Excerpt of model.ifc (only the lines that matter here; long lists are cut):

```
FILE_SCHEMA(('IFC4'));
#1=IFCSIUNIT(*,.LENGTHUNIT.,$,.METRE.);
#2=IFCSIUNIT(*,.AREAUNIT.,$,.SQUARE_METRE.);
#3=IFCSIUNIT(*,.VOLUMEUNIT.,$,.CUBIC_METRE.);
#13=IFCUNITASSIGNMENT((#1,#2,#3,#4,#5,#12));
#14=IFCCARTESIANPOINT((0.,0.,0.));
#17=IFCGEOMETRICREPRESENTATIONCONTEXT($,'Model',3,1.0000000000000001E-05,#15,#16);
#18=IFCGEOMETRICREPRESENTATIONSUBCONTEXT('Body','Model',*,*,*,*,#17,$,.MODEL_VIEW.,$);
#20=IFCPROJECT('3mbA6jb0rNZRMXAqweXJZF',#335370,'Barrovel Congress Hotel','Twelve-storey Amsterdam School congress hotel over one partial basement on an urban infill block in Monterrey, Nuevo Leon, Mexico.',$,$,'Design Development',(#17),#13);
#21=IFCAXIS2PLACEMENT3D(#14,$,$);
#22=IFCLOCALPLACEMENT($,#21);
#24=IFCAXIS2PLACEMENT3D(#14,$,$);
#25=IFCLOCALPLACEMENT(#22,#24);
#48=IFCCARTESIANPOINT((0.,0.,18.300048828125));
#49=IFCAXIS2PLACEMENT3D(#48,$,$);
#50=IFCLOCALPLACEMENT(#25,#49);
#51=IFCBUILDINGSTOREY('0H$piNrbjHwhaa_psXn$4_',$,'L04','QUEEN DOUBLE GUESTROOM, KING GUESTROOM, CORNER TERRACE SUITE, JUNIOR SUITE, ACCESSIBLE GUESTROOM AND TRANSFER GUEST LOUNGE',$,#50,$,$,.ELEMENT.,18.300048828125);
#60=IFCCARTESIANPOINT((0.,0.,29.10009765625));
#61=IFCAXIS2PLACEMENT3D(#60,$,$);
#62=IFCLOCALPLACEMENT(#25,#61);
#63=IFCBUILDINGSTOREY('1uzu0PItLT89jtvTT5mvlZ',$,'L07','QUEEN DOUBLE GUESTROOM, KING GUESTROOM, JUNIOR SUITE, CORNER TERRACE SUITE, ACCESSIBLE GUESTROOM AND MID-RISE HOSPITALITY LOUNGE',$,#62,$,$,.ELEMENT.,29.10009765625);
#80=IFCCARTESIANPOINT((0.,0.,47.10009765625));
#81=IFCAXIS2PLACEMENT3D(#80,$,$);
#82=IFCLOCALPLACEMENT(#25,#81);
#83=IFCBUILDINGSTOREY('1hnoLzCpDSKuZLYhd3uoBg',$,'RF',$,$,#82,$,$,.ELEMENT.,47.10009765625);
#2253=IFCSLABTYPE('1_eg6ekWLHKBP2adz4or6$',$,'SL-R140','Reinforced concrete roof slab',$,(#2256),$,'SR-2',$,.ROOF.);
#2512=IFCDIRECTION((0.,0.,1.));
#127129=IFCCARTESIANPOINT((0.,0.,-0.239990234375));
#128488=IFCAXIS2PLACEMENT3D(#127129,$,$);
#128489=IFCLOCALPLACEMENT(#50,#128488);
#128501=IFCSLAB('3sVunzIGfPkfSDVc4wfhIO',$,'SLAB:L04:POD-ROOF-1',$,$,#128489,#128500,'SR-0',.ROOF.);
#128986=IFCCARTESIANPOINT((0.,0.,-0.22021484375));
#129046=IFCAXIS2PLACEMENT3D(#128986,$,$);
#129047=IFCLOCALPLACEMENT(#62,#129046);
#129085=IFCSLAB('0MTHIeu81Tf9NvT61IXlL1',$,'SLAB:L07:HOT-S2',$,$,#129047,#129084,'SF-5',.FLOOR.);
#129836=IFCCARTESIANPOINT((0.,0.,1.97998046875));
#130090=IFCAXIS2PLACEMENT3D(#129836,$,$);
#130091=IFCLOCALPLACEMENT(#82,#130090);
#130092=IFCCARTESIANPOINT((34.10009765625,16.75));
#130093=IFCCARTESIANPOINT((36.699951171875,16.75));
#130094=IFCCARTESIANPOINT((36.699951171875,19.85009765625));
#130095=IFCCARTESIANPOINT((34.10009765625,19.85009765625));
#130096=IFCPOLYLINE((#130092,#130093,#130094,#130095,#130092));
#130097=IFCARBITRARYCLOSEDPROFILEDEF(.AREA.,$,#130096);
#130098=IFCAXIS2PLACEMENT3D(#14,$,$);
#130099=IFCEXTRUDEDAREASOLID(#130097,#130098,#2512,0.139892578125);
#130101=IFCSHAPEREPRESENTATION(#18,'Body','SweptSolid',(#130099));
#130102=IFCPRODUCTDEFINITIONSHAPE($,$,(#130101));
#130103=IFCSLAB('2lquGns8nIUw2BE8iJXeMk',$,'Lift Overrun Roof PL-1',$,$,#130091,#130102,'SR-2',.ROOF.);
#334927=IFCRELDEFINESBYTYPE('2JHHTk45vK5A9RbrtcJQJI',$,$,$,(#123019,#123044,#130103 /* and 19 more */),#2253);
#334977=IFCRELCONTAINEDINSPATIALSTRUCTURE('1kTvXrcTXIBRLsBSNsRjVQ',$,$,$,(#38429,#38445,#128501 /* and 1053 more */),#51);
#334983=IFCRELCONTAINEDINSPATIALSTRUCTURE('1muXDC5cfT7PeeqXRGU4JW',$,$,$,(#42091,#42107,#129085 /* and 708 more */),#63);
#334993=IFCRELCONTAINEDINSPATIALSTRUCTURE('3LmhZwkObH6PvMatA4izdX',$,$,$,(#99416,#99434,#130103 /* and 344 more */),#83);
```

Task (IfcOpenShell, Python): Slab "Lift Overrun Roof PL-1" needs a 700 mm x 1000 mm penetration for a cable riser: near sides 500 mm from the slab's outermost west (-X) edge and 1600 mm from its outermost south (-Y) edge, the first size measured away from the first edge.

```python
import numpy as np
import ifcopenshell
import ifcopenshell.api.feature
import ifcopenshell.api.geometry
import ifcopenshell.api.root
import ifcopenshell.geom
import ifcopenshell.util.placement
import ifcopenshell.util.representation
import ifcopenshell.util.shape
import ifcopenshell.util.unit

model = ifcopenshell.open("model.ifc")
unit_scale = ifcopenshell.util.unit.calculate_unit_scale(model)
settings = ifcopenshell.geom.settings()


def volume(element):
    """Net volume in cubic metres, openings subtracted."""
    shape = ifcopenshell.geom.create_shape(settings, element)
    return ifcopenshell.util.shape.get_volume(shape.geometry)


slab = model.by_guid("2lquGns8nIUw2BE8iJXeMk")
before = volume(slab)

# Extent in the slab's own axes, in metres. The edges named are its -X and -Y sides.
slab_shape = ifcopenshell.geom.create_shape(settings, slab)
vertices = ifcopenshell.util.shape.get_vertices(slab_shape.geometry)
x_min, y_min, bottom = vertices.min(axis=0)
top = vertices[:, 2].max()

opening = ifcopenshell.api.root.create_entity(model, ifc_class="IfcOpeningElement", name="Cable riser opening", predefined_type="OPENING")
context = ifcopenshell.util.representation.get_context(model, "Model", "Body", "MODEL_VIEW")
width, depth = 0.7, 1
outline = [(0.0, 0.0), (width, 0.0), (width, depth), (0.0, depth), (0.0, 0.0)]
# Overshoot both faces by 50 mm so the cut is clean.
shape = ifcopenshell.api.geometry.add_slab_representation(
    model, context=context, depth=top - bottom + 0.1, polyline=outline
)
ifcopenshell.api.geometry.assign_representation(model, product=opening, representation=shape)

matrix = ifcopenshell.util.placement.get_local_placement(slab.ObjectPlacement)
matrix[:, 3] = matrix @ np.append(np.array([x_min + 0.5, y_min + 1.6, bottom - 0.05]) / unit_scale, 1.0)
ifcopenshell.api.geometry.edit_object_placement(model, product=opening, matrix=matrix, is_si=False)
ifcopenshell.api.feature.add_feature(model, feature=opening, element=slab)

after = volume(slab)

print(f"slab volume {before:.3f} -> {after:.3f} m3")

model.write("model_v2.ifc")
```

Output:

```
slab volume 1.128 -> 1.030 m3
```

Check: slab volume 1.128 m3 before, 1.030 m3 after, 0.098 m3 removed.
